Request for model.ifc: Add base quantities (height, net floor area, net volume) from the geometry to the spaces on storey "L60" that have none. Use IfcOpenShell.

First a look at what the model holds.

```python
import ifcopenshell
import ifcopenshell.util.element
import ifcopenshell.util.unit

model = ifcopenshell.open("model.ifc")
print(model.schema)
for unit_type in ("LENGTHUNIT", "AREAUNIT", "VOLUMEUNIT"):
    print(unit_type, ifcopenshell.util.unit.calculate_unit_scale(model, unit_type))
storey = next(s for s in model.by_type("IfcBuildingStorey") if s.Name == "L60")
spaces = [e for e in ifcopenshell.util.element.get_decomposition(storey) if e.is_a("IfcSpace")]
for e in sorted(spaces, key=lambda e: e.id()):
    print(e.id(), e.is_a(), e.Name, list(ifcopenshell.util.element.get_psets(e, qtos_only=True)), sep=" | ")
```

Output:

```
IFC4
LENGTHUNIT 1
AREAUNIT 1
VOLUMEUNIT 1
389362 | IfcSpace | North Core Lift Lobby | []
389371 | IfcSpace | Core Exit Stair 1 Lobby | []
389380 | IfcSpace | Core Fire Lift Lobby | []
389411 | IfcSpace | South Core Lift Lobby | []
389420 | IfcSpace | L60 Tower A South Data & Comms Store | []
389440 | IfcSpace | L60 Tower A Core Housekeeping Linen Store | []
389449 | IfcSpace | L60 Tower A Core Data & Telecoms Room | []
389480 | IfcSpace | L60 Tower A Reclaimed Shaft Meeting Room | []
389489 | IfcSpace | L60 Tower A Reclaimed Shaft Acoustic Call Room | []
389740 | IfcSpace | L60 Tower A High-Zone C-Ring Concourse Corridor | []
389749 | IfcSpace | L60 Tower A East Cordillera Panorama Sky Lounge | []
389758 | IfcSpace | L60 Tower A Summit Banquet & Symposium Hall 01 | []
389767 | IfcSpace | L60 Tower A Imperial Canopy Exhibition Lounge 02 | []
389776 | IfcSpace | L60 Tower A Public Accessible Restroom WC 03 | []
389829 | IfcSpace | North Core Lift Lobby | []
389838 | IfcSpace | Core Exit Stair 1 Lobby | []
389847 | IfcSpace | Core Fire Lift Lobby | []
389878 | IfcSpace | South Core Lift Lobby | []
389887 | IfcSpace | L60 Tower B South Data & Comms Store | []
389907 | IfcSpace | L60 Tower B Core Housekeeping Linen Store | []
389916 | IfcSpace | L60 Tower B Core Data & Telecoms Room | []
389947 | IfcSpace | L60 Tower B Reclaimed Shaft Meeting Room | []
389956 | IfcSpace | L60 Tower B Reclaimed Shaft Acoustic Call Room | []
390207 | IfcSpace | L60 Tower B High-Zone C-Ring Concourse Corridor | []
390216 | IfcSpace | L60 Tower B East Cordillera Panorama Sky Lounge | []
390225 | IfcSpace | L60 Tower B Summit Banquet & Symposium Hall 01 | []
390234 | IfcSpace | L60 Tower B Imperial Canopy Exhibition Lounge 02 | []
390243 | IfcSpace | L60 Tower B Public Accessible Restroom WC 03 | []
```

```python
import ifcopenshell
import ifcopenshell.api.pset
import ifcopenshell.geom
import ifcopenshell.util.element
import ifcopenshell.util.shape
import ifcopenshell.util.unit

model = ifcopenshell.open("model.ifc")
unit_scale = ifcopenshell.util.unit.calculate_unit_scale(model)
area_scale = ifcopenshell.util.unit.calculate_unit_scale(model, "AREAUNIT")
volume_scale = ifcopenshell.util.unit.calculate_unit_scale(model, "VOLUMEUNIT")
settings = ifcopenshell.geom.settings()

storey = next(s for s in model.by_type("IfcBuildingStorey") if s.Name == "L60")
spaces = [e for e in ifcopenshell.util.element.get_decomposition(storey) if e.is_a("IfcSpace")]

for e in sorted(spaces, key=lambda e: e.id()):
    if ifcopenshell.util.element.get_psets(e, qtos_only=True, should_inherit=False):
        continue
    # Geometry comes back in metres, in the element's own axes.
    shape = ifcopenshell.geom.create_shape(settings, e)
    values = {
        "Height": ifcopenshell.util.shape.get_z(shape.geometry) / unit_scale,
        "NetFloorArea": ifcopenshell.util.shape.get_footprint_area(shape.geometry) / area_scale,
        "NetVolume": ifcopenshell.util.shape.get_volume(shape.geometry) / volume_scale,
    }
    qto = ifcopenshell.api.pset.add_qto(model, product=e, name="Qto_SpaceBaseQuantities")
    ifcopenshell.api.pset.edit_qto(model, qto=qto, properties=values)
    print(e.id(), {k: round(v, 3) for k, v in values.items()})

model.write("model_rev.ifc")
```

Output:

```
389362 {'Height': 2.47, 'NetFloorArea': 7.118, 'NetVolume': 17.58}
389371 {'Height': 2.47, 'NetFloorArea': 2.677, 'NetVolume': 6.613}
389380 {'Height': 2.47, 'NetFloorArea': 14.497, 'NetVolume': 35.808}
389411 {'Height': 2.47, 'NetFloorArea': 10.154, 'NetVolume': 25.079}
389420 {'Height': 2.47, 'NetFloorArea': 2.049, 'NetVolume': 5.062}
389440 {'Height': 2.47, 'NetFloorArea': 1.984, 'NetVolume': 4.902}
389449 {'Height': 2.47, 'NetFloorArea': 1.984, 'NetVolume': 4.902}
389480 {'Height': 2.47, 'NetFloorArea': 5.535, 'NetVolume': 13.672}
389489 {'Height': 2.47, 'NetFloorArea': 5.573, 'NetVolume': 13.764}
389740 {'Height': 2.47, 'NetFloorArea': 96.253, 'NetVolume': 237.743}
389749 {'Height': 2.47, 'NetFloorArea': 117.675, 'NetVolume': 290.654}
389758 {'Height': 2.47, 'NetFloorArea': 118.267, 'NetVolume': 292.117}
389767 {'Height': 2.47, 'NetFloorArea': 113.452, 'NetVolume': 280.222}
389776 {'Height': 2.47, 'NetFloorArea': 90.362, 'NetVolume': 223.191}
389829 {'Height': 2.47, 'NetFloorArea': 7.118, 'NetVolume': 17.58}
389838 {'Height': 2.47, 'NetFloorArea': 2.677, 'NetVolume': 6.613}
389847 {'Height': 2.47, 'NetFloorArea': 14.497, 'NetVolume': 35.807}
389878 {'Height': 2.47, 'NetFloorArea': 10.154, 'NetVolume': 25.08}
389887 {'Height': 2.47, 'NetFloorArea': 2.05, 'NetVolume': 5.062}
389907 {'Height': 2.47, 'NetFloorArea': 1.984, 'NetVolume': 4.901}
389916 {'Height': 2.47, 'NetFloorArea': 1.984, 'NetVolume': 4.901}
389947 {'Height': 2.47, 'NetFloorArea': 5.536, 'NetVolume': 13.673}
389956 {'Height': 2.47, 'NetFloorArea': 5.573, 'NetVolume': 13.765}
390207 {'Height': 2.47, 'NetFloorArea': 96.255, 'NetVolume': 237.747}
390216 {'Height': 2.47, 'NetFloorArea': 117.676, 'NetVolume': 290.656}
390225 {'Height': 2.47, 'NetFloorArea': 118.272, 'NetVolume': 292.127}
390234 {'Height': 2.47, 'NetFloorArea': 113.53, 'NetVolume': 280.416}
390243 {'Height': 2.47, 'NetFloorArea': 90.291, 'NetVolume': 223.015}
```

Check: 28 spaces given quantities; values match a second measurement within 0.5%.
